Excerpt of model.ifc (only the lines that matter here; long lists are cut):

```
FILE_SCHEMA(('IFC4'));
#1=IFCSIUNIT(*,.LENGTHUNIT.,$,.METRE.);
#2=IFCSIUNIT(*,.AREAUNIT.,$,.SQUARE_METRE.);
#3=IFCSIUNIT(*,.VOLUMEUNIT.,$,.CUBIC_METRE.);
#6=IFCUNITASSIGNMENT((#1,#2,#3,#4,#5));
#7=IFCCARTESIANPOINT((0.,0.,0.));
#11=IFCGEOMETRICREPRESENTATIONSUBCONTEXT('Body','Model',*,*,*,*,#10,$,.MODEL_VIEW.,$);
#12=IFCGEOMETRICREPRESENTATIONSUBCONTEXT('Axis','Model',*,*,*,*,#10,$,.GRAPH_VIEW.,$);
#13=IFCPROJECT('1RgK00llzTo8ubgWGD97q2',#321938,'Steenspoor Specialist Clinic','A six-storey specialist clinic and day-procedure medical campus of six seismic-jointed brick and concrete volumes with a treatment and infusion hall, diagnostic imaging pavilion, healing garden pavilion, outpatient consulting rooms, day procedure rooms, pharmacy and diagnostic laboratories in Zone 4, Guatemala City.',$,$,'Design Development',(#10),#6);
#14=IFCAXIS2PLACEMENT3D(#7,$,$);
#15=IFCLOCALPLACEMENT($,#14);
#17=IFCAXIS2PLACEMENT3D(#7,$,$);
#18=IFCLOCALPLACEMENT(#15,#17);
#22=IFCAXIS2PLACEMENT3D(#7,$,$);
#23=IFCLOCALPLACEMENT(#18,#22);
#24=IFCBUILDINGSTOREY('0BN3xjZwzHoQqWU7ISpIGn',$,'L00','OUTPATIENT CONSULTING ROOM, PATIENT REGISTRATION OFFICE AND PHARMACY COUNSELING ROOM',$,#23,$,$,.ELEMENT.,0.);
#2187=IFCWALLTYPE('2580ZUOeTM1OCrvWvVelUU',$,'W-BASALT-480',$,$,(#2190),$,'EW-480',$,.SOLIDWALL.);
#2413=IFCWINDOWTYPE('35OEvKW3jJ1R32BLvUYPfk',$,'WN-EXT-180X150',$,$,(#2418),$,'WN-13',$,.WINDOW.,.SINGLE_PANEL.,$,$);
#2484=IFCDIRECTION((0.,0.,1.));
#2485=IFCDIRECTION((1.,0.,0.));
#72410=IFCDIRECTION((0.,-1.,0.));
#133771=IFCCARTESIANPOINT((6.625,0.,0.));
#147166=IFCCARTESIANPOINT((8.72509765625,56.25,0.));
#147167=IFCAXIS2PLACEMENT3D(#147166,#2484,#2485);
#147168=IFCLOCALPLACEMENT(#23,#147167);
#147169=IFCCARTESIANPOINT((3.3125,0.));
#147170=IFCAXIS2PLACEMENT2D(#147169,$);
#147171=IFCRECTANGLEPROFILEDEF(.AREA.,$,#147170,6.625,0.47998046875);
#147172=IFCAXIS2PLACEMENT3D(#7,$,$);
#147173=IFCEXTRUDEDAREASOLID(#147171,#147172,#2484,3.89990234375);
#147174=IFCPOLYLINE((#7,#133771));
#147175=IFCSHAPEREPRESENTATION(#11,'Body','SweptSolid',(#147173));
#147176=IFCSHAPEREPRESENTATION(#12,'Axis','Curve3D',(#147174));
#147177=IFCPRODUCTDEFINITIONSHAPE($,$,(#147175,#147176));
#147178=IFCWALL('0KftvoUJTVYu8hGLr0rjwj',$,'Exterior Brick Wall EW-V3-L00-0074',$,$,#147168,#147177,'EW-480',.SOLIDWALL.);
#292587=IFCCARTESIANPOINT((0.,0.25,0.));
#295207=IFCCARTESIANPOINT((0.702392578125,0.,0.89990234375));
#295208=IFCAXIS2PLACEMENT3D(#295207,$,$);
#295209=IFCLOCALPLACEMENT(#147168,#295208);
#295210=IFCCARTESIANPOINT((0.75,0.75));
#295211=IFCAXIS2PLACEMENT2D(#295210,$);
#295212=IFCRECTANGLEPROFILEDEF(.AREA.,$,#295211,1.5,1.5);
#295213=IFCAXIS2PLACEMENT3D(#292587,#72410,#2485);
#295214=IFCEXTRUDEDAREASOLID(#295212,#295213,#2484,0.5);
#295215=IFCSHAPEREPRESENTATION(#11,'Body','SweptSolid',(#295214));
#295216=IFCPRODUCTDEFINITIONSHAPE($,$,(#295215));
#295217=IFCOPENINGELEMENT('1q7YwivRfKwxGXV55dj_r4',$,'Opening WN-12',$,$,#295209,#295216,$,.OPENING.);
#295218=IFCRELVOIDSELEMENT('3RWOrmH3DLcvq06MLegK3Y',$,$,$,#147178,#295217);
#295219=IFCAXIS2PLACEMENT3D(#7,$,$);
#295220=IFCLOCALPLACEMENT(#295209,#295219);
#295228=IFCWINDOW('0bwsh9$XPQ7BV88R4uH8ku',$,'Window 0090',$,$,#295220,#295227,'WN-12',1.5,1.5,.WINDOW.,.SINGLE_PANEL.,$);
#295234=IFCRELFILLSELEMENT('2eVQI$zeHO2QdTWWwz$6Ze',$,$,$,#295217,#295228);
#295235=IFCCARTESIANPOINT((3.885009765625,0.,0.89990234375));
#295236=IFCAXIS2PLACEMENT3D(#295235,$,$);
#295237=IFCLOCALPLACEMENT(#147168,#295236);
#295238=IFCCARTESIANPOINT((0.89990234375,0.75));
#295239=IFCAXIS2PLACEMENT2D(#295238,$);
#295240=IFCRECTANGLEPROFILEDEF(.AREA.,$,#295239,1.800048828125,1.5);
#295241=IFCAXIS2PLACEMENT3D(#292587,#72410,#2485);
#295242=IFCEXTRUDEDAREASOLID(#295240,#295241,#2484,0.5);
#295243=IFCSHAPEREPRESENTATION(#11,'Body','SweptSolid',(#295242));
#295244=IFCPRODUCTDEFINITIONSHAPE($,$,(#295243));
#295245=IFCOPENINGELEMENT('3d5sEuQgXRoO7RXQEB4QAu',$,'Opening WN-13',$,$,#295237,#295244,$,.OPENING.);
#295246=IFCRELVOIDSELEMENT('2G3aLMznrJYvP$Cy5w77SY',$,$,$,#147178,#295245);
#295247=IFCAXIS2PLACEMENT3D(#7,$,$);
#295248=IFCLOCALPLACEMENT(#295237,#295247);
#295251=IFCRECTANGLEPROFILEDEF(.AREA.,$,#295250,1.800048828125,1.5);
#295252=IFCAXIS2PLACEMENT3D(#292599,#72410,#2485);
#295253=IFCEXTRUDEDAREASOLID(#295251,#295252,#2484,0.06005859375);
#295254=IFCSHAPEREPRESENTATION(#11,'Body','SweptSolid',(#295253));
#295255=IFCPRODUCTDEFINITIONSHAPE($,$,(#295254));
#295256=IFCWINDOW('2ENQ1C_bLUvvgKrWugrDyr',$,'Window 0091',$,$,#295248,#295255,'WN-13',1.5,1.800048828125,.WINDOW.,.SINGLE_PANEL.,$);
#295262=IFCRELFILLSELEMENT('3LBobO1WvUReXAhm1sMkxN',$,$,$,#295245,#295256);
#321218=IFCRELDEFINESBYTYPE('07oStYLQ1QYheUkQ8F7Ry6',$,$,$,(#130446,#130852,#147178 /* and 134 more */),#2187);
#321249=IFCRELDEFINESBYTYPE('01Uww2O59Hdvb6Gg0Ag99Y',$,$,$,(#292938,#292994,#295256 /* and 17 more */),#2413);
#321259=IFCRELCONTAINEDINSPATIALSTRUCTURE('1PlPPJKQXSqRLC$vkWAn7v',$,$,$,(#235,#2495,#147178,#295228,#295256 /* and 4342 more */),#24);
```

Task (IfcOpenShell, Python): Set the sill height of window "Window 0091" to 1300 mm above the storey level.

```python
import numpy as np
import ifcopenshell
import ifcopenshell.api.geometry
import ifcopenshell.geom
import ifcopenshell.util.element
import ifcopenshell.util.placement
import ifcopenshell.util.shape
import ifcopenshell.util.unit

model = ifcopenshell.open("model.ifc")
unit_scale = ifcopenshell.util.unit.calculate_unit_scale(model)

window = model.by_guid("2ENQ1C_bLUvvgKrWugrDyr")
opening = window.FillsVoids[0].RelatingOpeningElement
storey = ifcopenshell.util.element.get_container(window, ifc_class="IfcBuildingStorey")
level = ifcopenshell.util.placement.get_local_placement(storey.ObjectPlacement)[2, 3]

# The opening's origin need not be at the sill, so measure its lowest point.
shape = ifcopenshell.geom.create_shape(ifcopenshell.geom.settings(), opening)
bottom = ifcopenshell.util.shape.get_shape_bottom_elevation(shape, shape.geometry) / unit_scale
dz = level + 1.3 / unit_scale - bottom

shift = np.array([0.0, 0.0, dz])
# The window is placed relative to its opening, so it follows when the opening moves.
matrix = ifcopenshell.util.placement.get_local_placement(opening.ObjectPlacement)
matrix[:3, 3] += shift
ifcopenshell.api.geometry.edit_object_placement(
    model, product=opening, matrix=matrix, is_si=False, should_transform_children=True
)

print(f"moved by {dz * unit_scale:+.3f} m")

model.write("model-out.ifc")
```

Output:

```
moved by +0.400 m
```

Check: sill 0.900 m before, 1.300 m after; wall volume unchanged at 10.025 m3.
